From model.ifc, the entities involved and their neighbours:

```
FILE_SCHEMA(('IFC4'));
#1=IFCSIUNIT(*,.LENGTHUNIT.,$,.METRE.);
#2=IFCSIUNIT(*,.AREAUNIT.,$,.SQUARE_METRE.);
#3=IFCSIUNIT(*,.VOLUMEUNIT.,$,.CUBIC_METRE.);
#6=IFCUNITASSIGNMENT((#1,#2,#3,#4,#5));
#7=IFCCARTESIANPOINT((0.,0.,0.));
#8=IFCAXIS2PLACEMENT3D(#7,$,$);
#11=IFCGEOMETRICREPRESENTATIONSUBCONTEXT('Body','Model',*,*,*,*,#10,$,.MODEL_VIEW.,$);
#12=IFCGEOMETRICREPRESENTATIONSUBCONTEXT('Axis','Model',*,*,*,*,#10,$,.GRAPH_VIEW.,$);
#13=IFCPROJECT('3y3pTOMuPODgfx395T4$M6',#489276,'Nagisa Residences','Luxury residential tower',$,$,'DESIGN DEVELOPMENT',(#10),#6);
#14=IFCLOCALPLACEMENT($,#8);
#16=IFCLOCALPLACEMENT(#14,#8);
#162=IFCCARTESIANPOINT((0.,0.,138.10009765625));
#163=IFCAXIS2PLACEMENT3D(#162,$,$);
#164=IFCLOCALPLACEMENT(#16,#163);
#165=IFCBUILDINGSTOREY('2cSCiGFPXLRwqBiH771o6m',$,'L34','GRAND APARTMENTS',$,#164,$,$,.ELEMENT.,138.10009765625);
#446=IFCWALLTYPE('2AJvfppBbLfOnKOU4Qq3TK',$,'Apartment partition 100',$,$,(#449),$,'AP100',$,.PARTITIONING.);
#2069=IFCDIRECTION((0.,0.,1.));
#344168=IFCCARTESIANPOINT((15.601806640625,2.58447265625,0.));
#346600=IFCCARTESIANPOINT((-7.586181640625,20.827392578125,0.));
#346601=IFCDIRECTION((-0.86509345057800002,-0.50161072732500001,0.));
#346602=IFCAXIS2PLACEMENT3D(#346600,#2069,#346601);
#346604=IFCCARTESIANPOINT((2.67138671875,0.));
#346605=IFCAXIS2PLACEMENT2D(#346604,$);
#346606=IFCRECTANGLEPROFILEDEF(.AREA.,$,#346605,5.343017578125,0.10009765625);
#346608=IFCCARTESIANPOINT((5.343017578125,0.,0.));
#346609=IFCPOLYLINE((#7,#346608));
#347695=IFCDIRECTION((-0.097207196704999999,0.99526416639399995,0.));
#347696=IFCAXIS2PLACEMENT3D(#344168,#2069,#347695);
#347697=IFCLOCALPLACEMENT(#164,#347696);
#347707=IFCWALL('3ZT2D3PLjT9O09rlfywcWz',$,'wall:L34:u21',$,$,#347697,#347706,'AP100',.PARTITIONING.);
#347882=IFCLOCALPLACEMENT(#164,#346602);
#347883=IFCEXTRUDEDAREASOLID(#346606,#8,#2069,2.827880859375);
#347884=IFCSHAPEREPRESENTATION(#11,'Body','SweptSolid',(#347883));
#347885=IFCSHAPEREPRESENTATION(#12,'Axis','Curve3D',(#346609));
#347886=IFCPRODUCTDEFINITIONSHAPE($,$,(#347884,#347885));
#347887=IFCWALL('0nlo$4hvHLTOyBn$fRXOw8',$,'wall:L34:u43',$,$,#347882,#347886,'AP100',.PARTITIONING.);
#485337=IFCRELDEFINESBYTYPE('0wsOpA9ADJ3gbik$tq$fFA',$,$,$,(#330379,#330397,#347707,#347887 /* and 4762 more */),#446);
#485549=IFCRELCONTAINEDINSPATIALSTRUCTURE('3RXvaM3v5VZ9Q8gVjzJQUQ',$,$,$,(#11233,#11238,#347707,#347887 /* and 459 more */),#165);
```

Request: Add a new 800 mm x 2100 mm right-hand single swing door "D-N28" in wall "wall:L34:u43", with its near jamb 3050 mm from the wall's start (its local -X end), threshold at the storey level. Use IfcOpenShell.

```python
import numpy as np
import ifcopenshell
import ifcopenshell.api.feature
import ifcopenshell.api.geometry
import ifcopenshell.api.root
import ifcopenshell.api.spatial
import ifcopenshell.geom
import ifcopenshell.util.element
import ifcopenshell.util.placement
import ifcopenshell.util.representation
import ifcopenshell.util.shape
import ifcopenshell.util.unit

model = ifcopenshell.open("model.ifc")
unit_scale = ifcopenshell.util.unit.calculate_unit_scale(model)
settings = ifcopenshell.geom.settings()


def volume(element):
    """Net volume in cubic metres, openings subtracted."""
    shape = ifcopenshell.geom.create_shape(settings, element)
    return ifcopenshell.util.shape.get_volume(shape.geometry)


wall = model.by_guid("0nlo$4hvHLTOyBn$fRXOw8")
storey = ifcopenshell.util.element.get_container(wall, ifc_class="IfcBuildingStorey")
context = ifcopenshell.util.representation.get_context(model, "Model", "Body", "MODEL_VIEW")
before = volume(wall)

width, height, from_end, sill = 0.8, 2.1, 3.05, 0.0  # metres

# The wall runs along its own X axis, and the end named is its -X end.
wall_shape = ifcopenshell.geom.create_shape(settings, wall)
x, y, z = ifcopenshell.util.shape.get_vertices(wall_shape.geometry).T
start = x.min() + from_end
face, thickness = float(y.min()), float(y.max() - y.min())
wall_matrix = ifcopenshell.util.placement.get_local_placement(wall.ObjectPlacement)
level = ifcopenshell.util.placement.get_local_placement(storey.ObjectPlacement)[2, 3]


def in_wall(x, y):
    """Placement at x, y metres in the wall's axes, at sill height."""
    matrix = wall_matrix.copy()
    matrix[:, 3] = wall_matrix @ np.array([x / unit_scale, y / unit_scale, 0.0, 1.0])
    matrix[2, 3] = level + sill / unit_scale
    return matrix


# Opening: a box that overshoots both wall faces by 50 mm.
opening = ifcopenshell.api.root.create_entity(model, ifc_class="IfcOpeningElement", predefined_type="OPENING")
box = ifcopenshell.api.geometry.add_wall_representation(
    model, context=context, length=width, height=height, thickness=thickness + 0.1
)
ifcopenshell.api.geometry.assign_representation(model, product=opening, representation=box)
ifcopenshell.api.geometry.edit_object_placement(model, product=opening, matrix=in_wall(start, face - 0.05), is_si=False)
ifcopenshell.api.feature.add_feature(model, feature=opening, element=wall)

door = ifcopenshell.api.root.create_entity(model, ifc_class="IfcDoor", name="D-N28", predefined_type="DOOR")
door.OverallWidth, door.OverallHeight = width / unit_scale, height / unit_scale
door.OperationType = "SINGLE_SWING_RIGHT"
body = ifcopenshell.api.geometry.add_door_representation(
    model,
    context=context,
    overall_width=door.OverallWidth,
    overall_height=door.OverallHeight,
    operation_type="SINGLE_SWING_RIGHT",
    lining_properties={"LiningDepth": thickness / unit_scale, "ThresholdDepth": thickness / unit_scale},
)
ifcopenshell.api.geometry.assign_representation(model, product=door, representation=body)
ifcopenshell.api.spatial.assign_container(model, products=[door], relating_structure=storey)
ifcopenshell.api.feature.add_filling(model, opening=opening, element=door)

# The lining spans the wall, so the door starts at the wall face.
ifcopenshell.api.geometry.edit_object_placement(model, product=door, matrix=in_wall(start, face), is_si=False)

after = volume(wall)

print(f"wall volume {before:.3f} -> {after:.3f} m3")

model.write("model-out.ifc")
```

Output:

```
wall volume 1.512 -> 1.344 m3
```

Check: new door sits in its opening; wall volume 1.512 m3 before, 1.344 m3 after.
